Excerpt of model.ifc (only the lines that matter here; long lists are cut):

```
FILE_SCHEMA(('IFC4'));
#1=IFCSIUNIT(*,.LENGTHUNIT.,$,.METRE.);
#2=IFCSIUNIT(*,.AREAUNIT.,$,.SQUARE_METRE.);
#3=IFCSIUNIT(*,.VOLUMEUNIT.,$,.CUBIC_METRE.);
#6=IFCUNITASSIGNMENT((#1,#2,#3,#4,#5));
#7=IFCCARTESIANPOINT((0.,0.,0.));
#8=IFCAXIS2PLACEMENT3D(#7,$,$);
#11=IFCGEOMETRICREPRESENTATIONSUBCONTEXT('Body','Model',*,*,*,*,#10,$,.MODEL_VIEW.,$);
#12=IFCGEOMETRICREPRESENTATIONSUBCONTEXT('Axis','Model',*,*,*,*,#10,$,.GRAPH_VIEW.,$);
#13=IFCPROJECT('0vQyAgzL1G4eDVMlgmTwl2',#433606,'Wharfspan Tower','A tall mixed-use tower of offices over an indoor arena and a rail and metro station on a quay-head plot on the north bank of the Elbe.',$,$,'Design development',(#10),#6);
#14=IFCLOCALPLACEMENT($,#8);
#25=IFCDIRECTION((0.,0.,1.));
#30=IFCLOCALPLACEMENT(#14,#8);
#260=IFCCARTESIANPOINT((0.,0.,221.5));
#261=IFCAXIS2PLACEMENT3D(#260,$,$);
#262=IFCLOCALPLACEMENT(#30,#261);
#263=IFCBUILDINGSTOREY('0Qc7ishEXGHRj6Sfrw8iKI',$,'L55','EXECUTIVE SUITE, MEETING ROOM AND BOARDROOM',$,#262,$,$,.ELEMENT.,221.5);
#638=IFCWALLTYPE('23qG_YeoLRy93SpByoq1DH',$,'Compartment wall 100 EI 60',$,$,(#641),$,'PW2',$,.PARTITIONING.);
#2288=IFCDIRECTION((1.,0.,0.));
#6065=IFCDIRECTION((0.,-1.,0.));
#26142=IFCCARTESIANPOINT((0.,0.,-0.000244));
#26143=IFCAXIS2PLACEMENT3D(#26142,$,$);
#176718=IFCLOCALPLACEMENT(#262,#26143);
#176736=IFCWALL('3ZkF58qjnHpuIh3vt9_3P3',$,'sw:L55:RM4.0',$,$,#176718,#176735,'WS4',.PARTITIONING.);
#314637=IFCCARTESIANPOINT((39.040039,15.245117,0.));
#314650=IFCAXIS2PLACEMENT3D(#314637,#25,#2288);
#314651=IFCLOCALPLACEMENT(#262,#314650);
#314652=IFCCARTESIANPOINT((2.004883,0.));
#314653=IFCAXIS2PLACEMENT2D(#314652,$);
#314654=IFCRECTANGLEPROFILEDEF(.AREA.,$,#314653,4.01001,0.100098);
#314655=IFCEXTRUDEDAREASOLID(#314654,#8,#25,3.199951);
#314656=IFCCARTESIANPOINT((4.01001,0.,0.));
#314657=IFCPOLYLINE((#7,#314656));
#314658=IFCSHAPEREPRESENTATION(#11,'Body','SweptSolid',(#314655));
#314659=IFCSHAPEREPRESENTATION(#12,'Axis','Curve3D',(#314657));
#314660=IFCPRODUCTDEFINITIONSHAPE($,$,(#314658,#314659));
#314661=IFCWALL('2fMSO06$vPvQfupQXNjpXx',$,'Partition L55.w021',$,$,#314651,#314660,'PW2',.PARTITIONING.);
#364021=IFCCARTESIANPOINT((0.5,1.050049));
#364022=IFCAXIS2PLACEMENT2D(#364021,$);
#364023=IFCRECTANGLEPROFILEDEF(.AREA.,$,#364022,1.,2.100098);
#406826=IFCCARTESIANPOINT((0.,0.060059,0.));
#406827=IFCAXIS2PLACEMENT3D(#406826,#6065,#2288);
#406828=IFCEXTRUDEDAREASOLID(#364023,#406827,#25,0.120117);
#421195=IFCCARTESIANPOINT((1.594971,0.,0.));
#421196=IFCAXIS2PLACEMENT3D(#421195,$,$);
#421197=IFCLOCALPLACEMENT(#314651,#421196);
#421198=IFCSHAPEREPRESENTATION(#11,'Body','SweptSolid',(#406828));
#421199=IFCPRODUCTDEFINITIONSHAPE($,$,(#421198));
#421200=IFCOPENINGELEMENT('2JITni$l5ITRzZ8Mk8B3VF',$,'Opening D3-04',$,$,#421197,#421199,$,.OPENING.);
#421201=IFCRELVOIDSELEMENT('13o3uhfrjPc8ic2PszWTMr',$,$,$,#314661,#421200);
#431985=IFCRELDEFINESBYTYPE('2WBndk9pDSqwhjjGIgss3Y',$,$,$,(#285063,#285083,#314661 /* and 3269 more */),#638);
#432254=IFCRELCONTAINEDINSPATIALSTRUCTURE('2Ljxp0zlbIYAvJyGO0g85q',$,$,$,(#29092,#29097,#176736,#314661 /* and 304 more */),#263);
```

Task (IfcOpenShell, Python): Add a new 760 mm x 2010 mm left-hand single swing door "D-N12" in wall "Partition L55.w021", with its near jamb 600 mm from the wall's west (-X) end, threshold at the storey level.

```python
import numpy as np
import ifcopenshell
import ifcopenshell.api.feature
import ifcopenshell.api.geometry
import ifcopenshell.api.root
import ifcopenshell.api.spatial
import ifcopenshell.geom
import ifcopenshell.util.element
import ifcopenshell.util.placement
import ifcopenshell.util.representation
import ifcopenshell.util.shape
import ifcopenshell.util.unit

model = ifcopenshell.open("model.ifc")
unit_scale = ifcopenshell.util.unit.calculate_unit_scale(model)
settings = ifcopenshell.geom.settings()


def volume(element):
    """Net volume in cubic metres, openings subtracted."""
    shape = ifcopenshell.geom.create_shape(settings, element)
    return ifcopenshell.util.shape.get_volume(shape.geometry)


wall = model.by_guid("2fMSO06$vPvQfupQXNjpXx")
storey = ifcopenshell.util.element.get_container(wall, ifc_class="IfcBuildingStorey")
context = ifcopenshell.util.representation.get_context(model, "Model", "Body", "MODEL_VIEW")
before = volume(wall)

width, height, from_end, sill = 0.76, 2.01, 0.6, 0.0  # metres

# The wall runs along its own X axis, and the end named is its -X end.
wall_shape = ifcopenshell.geom.create_shape(settings, wall)
x, y, z = ifcopenshell.util.shape.get_vertices(wall_shape.geometry).T
start = x.min() + from_end
face, thickness = float(y.min()), float(y.max() - y.min())
wall_matrix = ifcopenshell.util.placement.get_local_placement(wall.ObjectPlacement)
level = ifcopenshell.util.placement.get_local_placement(storey.ObjectPlacement)[2, 3]


def in_wall(x, y):
    """Placement at x, y metres in the wall's axes, at sill height."""
    matrix = wall_matrix.copy()
    matrix[:, 3] = wall_matrix @ np.array([x / unit_scale, y / unit_scale, 0.0, 1.0])
    matrix[2, 3] = level + sill / unit_scale
    return matrix


# Opening: a box that overshoots both wall faces by 50 mm.
opening = ifcopenshell.api.root.create_entity(model, ifc_class="IfcOpeningElement", predefined_type="OPENING")
box = ifcopenshell.api.geometry.add_wall_representation(
    model, context=context, length=width, height=height, thickness=thickness + 0.1
)
ifcopenshell.api.geometry.assign_representation(model, product=opening, representation=box)
ifcopenshell.api.geometry.edit_object_placement(model, product=opening, matrix=in_wall(start, face - 0.05), is_si=False)
ifcopenshell.api.feature.add_feature(model, feature=opening, element=wall)

door = ifcopenshell.api.root.create_entity(model, ifc_class="IfcDoor", name="D-N12", predefined_type="DOOR")
door.OverallWidth, door.OverallHeight = width / unit_scale, height / unit_scale
door.OperationType = "SINGLE_SWING_LEFT"
body = ifcopenshell.api.geometry.add_door_representation(
    model,
    context=context,
    overall_width=door.OverallWidth,
    overall_height=door.OverallHeight,
    operation_type="SINGLE_SWING_LEFT",
    lining_properties={"LiningDepth": thickness / unit_scale, "ThresholdDepth": thickness / unit_scale},
)
ifcopenshell.api.geometry.assign_representation(model, product=door, representation=body)
ifcopenshell.api.spatial.assign_container(model, products=[door], relating_structure=storey)
ifcopenshell.api.feature.add_filling(model, opening=opening, element=door)

# The lining spans the wall, so the door starts at the wall face.
ifcopenshell.api.geometry.edit_object_placement(model, product=door, matrix=in_wall(start, face), is_si=False)

after = volume(wall)

print(f"wall volume {before:.3f} -> {after:.3f} m3")

model.write("model_edited.ifc")
```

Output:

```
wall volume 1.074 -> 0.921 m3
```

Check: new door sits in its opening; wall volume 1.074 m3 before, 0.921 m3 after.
